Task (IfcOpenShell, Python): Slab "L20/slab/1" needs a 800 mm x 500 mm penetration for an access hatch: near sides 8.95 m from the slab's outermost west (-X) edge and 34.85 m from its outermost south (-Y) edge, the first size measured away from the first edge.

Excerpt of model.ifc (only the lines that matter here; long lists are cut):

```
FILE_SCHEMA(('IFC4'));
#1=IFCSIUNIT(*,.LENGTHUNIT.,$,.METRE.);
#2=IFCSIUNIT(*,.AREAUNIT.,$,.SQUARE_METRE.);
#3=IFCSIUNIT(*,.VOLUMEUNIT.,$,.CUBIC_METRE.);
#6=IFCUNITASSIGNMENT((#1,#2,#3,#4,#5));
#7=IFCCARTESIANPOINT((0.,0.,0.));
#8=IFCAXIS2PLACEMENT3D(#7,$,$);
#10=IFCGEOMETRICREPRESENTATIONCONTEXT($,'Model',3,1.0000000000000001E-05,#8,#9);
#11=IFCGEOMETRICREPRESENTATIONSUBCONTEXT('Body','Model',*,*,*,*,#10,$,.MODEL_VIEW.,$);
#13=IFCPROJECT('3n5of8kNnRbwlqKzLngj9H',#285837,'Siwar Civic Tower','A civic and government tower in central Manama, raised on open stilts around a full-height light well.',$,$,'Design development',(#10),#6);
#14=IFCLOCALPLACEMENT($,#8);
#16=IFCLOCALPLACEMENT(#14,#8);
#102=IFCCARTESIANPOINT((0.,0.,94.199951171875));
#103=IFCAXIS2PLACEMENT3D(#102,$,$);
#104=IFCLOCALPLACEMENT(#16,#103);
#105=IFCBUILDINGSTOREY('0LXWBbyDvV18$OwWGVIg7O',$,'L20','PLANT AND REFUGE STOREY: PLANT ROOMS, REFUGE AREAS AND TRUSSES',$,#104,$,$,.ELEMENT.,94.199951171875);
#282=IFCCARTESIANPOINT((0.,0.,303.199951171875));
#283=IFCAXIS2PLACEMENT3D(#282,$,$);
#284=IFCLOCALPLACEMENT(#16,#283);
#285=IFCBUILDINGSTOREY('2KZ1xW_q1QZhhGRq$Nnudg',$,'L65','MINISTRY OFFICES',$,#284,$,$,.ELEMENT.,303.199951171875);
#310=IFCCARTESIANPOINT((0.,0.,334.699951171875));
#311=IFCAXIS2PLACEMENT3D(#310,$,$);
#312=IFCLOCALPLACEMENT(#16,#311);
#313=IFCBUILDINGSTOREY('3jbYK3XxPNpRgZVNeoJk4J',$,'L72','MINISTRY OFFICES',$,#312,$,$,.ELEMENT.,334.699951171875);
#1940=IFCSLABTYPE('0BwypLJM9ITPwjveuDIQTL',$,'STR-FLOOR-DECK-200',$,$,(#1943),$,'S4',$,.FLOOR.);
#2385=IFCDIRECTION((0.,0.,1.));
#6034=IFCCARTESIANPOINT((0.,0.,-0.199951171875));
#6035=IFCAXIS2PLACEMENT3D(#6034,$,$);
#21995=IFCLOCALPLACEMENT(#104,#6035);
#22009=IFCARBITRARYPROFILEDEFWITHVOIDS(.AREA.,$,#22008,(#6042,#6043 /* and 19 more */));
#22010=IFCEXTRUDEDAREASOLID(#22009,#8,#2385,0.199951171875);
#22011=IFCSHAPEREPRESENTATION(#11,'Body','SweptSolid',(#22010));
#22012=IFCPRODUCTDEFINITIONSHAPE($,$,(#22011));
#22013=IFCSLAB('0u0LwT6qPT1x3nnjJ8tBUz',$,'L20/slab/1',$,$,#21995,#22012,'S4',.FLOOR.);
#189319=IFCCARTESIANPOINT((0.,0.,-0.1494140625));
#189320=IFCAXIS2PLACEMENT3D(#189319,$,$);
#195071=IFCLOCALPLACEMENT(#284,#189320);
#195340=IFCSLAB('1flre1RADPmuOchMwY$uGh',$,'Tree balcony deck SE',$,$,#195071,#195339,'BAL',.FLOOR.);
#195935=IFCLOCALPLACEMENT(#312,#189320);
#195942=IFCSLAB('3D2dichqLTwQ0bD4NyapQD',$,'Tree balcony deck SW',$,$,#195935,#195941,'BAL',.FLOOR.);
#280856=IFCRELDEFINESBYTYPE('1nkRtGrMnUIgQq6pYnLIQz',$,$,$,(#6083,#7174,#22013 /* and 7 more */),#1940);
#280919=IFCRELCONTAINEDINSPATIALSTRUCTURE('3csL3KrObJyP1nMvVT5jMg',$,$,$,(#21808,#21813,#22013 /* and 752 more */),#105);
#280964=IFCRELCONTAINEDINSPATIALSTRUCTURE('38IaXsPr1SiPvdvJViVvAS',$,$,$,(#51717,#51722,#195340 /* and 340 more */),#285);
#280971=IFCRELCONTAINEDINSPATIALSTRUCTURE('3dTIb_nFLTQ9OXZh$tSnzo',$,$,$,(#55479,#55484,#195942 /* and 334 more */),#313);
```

```python
import numpy as np
import ifcopenshell
import ifcopenshell.api.feature
import ifcopenshell.api.geometry
import ifcopenshell.api.root
import ifcopenshell.geom
import ifcopenshell.util.placement
import ifcopenshell.util.representation
import ifcopenshell.util.shape
import ifcopenshell.util.unit

model = ifcopenshell.open("model.ifc")
unit_scale = ifcopenshell.util.unit.calculate_unit_scale(model)
settings = ifcopenshell.geom.settings()


def volume(element):
    """Net volume in cubic metres, openings subtracted."""
    shape = ifcopenshell.geom.create_shape(settings, element)
    return ifcopenshell.util.shape.get_volume(shape.geometry)


slab = model.by_guid("0u0LwT6qPT1x3nnjJ8tBUz")
before = volume(slab)

# Extent in the slab's own axes, in metres. The edges named are its -X and -Y sides.
slab_shape = ifcopenshell.geom.create_shape(settings, slab)
vertices = ifcopenshell.util.shape.get_vertices(slab_shape.geometry)
x_min, y_min, bottom = vertices.min(axis=0)
top = vertices[:, 2].max()

opening = ifcopenshell.api.root.create_entity(model, ifc_class="IfcOpeningElement", name="Access hatch opening", predefined_type="OPENING")
context = ifcopenshell.util.representation.get_context(model, "Model", "Body", "MODEL_VIEW")
width, depth = 0.8, 0.5
outline = [(0.0, 0.0), (width, 0.0), (width, depth), (0.0, depth), (0.0, 0.0)]
# Overshoot both faces by 50 mm so the cut is clean.
shape = ifcopenshell.api.geometry.add_slab_representation(
    model, context=context, depth=top - bottom + 0.1, polyline=outline
)
ifcopenshell.api.geometry.assign_representation(model, product=opening, representation=shape)

matrix = ifcopenshell.util.placement.get_local_placement(slab.ObjectPlacement)
matrix[:, 3] = matrix @ np.append(np.array([x_min + 8.95, y_min + 34.85, bottom - 0.05]) / unit_scale, 1.0)
ifcopenshell.api.geometry.edit_object_placement(model, product=opening, matrix=matrix, is_si=False)
ifcopenshell.api.feature.add_feature(model, feature=opening, element=slab)

after = volume(slab)

print(f"slab volume {before:.3f} -> {after:.3f} m3")

model.write("model_updated.ifc")
```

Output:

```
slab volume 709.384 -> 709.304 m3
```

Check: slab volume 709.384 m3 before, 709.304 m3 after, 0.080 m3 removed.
